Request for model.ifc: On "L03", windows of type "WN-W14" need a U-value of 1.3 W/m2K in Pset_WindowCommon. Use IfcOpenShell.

First a look at what the model holds.

```python
import ifcopenshell
import ifcopenshell.util.element

model = ifcopenshell.open("model.ifc")
print(model.schema)
storey = next(s for s in model.by_type("IfcBuildingStorey") if s.Name == "L03")
windows = [e for e in ifcopenshell.util.element.get_decomposition(storey) if e.is_a("IfcWindow")]
seen = {}
for e in windows:
    element_type = ifcopenshell.util.element.get_type(e)
    key = (element_type.Name if element_type != e and element_type else None, ifcopenshell.util.element.get_pset(e, "Pset_WindowCommon", "ThermalTransmittance"))
    seen[key] = seen.get(key, 0) + 1
for (name, value), count in sorted(seen.items(), key=str):
    print(count, "x", name, "|", value)
```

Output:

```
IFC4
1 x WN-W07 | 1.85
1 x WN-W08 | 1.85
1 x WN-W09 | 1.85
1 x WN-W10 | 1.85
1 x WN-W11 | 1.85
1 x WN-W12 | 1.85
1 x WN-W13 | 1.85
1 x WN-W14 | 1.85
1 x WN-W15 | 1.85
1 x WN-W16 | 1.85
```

```python
import ifcopenshell
import ifcopenshell.api.pset
import ifcopenshell.util.element

model = ifcopenshell.open("model.ifc")

storey = next(s for s in model.by_type("IfcBuildingStorey") if s.Name == "L03")
windows = [e for e in ifcopenshell.util.element.get_decomposition(storey) if e.is_a("IfcWindow")]

count = 0
for e in windows:
    element_type = ifcopenshell.util.element.get_type(e)
    if element_type in (None, e) or element_type.Name != "WN-W14":
        continue
    # add_pset returns the element's existing set when there is one.
    pset = ifcopenshell.api.pset.add_pset(model, product=e, name="Pset_WindowCommon")
    ifcopenshell.api.pset.edit_pset(model, pset=pset, properties={"ThermalTransmittance": 1.3})
    count += 1

print(count, "windows updated")

model.write("model_v2.ifc")
```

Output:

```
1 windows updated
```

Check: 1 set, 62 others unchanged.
